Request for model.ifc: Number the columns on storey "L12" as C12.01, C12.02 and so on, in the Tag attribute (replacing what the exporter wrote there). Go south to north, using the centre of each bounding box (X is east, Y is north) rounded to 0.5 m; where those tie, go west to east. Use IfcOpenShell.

First a look at what the model holds.

```python
import ifcopenshell
import ifcopenshell.util.element
import ifcopenshell.util.placement

model = ifcopenshell.open("model.ifc")
print(model.schema)
storey = next(s for s in model.by_type("IfcBuildingStorey") if s.Name == "L12")
columns = [e for e in ifcopenshell.util.element.get_decomposition(storey) if e.is_a("IfcColumn")]
for e in sorted(columns, key=lambda e: e.id()):
    origin = ifcopenshell.util.placement.get_local_placement(e.ObjectPlacement)[:3, 3]
    print(e.id(), e.Tag, e.Name, origin.round(2) + 0.0, sep=" | ")
```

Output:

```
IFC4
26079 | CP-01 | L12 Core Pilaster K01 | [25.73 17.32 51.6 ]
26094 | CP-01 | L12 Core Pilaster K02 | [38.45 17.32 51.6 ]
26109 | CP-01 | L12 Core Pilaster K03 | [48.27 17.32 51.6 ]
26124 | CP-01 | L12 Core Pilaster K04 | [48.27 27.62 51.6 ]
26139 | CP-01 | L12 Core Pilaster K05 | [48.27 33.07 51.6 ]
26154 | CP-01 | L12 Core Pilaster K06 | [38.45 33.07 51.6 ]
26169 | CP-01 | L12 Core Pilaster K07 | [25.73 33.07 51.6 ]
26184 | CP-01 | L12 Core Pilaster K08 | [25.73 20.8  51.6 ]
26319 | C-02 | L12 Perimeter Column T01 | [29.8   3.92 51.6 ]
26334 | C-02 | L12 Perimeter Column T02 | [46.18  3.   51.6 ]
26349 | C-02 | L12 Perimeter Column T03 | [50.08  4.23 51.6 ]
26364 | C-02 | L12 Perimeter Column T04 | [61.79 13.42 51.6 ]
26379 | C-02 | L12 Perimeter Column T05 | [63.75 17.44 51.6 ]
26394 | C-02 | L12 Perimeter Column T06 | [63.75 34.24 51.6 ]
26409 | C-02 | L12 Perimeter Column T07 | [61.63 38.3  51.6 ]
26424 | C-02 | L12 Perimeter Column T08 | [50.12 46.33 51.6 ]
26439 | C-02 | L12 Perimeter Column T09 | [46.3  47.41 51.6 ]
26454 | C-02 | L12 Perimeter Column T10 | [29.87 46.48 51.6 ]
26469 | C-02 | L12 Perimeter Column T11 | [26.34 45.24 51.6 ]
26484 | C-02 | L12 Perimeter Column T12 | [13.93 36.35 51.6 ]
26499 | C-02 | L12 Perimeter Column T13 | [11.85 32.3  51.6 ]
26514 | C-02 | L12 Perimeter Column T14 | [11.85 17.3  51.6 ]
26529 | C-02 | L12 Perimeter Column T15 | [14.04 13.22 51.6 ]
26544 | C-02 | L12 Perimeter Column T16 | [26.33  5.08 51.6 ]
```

```python
import ifcopenshell
import ifcopenshell.geom
import ifcopenshell.util.element
import ifcopenshell.util.shape

model = ifcopenshell.open("model.ifc")
settings = ifcopenshell.geom.settings()
settings.set("use-world-coords", True)


def centre(element):
    shape = ifcopenshell.geom.create_shape(settings, element)
    return ifcopenshell.util.shape.get_bbox_centroid(shape.geometry)


storey = next(s for s in model.by_type("IfcBuildingStorey") if s.Name == "L12")
columns = [e for e in ifcopenshell.util.element.get_decomposition(storey) if e.is_a("IfcColumn")]

# Insertion points can sit at a corner or the storey origin, so sort by the geometry (in metres).
centres = {e: centre(e) for e in columns}
columns.sort(key=lambda e: (round(centres[e][1] / 0.5), centres[e][0]))

for i, e in enumerate(columns, start=1):
    number = f"C12.{i:02d}"
    e.Tag = number
    print(e.id(), number)

model.write("model_rev.ifc")
```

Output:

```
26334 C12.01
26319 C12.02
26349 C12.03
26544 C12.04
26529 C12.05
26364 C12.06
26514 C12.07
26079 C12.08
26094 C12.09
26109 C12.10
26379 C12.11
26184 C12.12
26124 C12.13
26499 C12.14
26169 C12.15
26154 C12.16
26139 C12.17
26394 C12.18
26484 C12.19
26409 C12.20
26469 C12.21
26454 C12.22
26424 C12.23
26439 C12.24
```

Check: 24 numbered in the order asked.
